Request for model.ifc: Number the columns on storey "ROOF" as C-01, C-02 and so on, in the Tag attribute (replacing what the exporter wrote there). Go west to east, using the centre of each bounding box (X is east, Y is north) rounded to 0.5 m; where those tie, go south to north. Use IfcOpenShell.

First a look at what the model holds.

```python
import ifcopenshell
import ifcopenshell.util.element
import ifcopenshell.util.placement

model = ifcopenshell.open("model.ifc")
print(model.schema)
storey = next(s for s in model.by_type("IfcBuildingStorey") if s.Name == "ROOF")
columns = [e for e in ifcopenshell.util.element.get_decomposition(storey) if e.is_a("IfcColumn")]
for e in sorted(columns, key=lambda e: e.id()):
    origin = ifcopenshell.util.placement.get_local_placement(e.ObjectPlacement)[:3, 3]
    print(e.id(), e.Tag, e.Name, origin.round(2) + 0.0, sep=" | ")
```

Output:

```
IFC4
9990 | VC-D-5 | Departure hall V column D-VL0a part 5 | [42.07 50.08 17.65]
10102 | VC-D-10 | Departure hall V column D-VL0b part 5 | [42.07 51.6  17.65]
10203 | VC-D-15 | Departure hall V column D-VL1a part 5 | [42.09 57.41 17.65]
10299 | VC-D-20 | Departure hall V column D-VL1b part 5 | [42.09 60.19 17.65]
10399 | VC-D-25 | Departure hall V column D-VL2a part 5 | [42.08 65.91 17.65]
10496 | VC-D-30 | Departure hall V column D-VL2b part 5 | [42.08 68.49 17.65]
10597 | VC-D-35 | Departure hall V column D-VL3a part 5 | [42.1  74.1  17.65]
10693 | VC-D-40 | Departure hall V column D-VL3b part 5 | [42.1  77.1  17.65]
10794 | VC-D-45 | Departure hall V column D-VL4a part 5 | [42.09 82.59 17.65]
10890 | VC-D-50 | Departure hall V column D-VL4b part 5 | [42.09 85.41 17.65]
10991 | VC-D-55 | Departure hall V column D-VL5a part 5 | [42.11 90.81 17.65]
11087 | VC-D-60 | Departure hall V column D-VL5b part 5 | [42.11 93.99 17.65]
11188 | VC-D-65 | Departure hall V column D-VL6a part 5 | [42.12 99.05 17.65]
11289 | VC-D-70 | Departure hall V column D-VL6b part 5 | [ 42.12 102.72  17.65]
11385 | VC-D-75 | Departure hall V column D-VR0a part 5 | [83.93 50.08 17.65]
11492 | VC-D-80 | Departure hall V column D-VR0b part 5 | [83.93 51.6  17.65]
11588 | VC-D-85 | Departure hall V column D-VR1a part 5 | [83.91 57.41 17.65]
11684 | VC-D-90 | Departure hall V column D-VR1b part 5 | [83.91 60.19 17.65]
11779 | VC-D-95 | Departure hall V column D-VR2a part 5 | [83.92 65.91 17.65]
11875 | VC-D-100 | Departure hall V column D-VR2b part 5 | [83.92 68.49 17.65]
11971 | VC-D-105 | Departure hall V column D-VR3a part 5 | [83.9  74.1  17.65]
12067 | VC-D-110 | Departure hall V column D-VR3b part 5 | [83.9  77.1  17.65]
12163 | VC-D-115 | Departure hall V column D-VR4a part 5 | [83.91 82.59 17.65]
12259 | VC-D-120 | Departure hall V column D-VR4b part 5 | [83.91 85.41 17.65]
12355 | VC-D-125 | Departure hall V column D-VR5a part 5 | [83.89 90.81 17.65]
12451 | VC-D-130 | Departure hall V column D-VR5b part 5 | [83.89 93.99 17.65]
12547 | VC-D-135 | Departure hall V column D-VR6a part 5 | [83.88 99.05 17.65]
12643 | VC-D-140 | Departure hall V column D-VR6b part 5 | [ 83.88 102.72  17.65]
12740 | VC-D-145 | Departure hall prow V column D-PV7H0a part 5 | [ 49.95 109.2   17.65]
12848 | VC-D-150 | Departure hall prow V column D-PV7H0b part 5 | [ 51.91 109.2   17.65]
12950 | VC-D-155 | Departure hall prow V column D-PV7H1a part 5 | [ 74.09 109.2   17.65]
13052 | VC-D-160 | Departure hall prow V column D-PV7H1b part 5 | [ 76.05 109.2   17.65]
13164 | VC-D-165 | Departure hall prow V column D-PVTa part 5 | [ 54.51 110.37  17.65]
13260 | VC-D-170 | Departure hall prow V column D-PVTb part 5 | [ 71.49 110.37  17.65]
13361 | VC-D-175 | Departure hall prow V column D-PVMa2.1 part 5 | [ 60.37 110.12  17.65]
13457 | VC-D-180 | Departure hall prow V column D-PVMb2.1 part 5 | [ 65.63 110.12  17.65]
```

```python
import ifcopenshell
import ifcopenshell.geom
import ifcopenshell.util.element
import ifcopenshell.util.shape

model = ifcopenshell.open("model.ifc")
settings = ifcopenshell.geom.settings()
settings.set("use-world-coords", True)


def centre(element):
    shape = ifcopenshell.geom.create_shape(settings, element)
    return ifcopenshell.util.shape.get_bbox_centroid(shape.geometry)


storey = next(s for s in model.by_type("IfcBuildingStorey") if s.Name == "ROOF")
columns = [e for e in ifcopenshell.util.element.get_decomposition(storey) if e.is_a("IfcColumn")]

# Insertion points can sit at a corner or the storey origin, so sort by the geometry (in metres).
centres = {e: centre(e) for e in columns}
columns.sort(key=lambda e: (round(centres[e][0] / 0.5), centres[e][1]))

for i, e in enumerate(columns, start=1):
    number = f"C-{i:02d}"
    e.Tag = number
    print(e.id(), number)

model.write("model_edited.ifc")
```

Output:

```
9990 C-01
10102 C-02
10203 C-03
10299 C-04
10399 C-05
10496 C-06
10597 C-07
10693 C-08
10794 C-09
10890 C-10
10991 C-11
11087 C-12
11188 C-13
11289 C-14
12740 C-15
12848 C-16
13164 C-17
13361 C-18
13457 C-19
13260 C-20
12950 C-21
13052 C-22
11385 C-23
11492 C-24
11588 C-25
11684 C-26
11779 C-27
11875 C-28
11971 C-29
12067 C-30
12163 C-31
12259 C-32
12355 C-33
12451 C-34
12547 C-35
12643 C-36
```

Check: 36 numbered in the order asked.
